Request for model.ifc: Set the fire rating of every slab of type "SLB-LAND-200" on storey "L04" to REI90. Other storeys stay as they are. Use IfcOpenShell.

First a look at what the model holds.

```python
import ifcopenshell
import ifcopenshell.util.element

model = ifcopenshell.open("model.ifc")
print(model.schema)
storey = next(s for s in model.by_type("IfcBuildingStorey") if s.Name == "L04")
slabs = [e for e in ifcopenshell.util.element.get_decomposition(storey) if e.is_a("IfcSlab")]
seen = {}
for e in slabs:
    element_type = ifcopenshell.util.element.get_type(e)
    key = (element_type.Name if element_type != e and element_type else None, ifcopenshell.util.element.get_pset(e, "Pset_SlabCommon", "FireRating"))
    seen[key] = seen.get(key, 0) + 1
for (name, value), count in sorted(seen.items(), key=str):
    print(count, "x", name, "|", value)
```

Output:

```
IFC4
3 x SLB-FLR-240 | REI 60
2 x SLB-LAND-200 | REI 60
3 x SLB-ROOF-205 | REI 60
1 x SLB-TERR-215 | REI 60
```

```python
import ifcopenshell
import ifcopenshell.api.pset
import ifcopenshell.util.element

model = ifcopenshell.open("model.ifc")

storey = next(s for s in model.by_type("IfcBuildingStorey") if s.Name == "L04")
slabs = [e for e in ifcopenshell.util.element.get_decomposition(storey) if e.is_a("IfcSlab")]

count = 0
for e in slabs:
    element_type = ifcopenshell.util.element.get_type(e)
    if element_type in (None, e) or element_type.Name != "SLB-LAND-200":
        continue
    # add_pset returns the element's existing set when there is one.
    pset = ifcopenshell.api.pset.add_pset(model, product=e, name="Pset_SlabCommon")
    ifcopenshell.api.pset.edit_pset(model, pset=pset, properties={"FireRating": "REI90"})
    count += 1

print(count, "slabs updated")

model.write("model-out.ifc")
```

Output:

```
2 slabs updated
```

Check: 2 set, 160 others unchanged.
